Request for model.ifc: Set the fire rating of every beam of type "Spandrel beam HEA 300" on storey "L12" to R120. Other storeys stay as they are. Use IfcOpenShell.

First a look at what the model holds.

```python
import ifcopenshell
import ifcopenshell.util.element

model = ifcopenshell.open("model.ifc")
print(model.schema)
storey = next(s for s in model.by_type("IfcBuildingStorey") if s.Name == "L12")
beams = [e for e in ifcopenshell.util.element.get_decomposition(storey) if e.is_a("IfcBeam")]
seen = {}
for e in beams:
    element_type = ifcopenshell.util.element.get_type(e)
    key = (element_type.Name if element_type != e and element_type else None, ifcopenshell.util.element.get_pset(e, "Pset_BeamCommon", "FireRating"))
    seen[key] = seen.get(key, 0) + 1
for (name, value), count in sorted(seen.items(), key=str):
    print(count, "x", name, "|", value)
```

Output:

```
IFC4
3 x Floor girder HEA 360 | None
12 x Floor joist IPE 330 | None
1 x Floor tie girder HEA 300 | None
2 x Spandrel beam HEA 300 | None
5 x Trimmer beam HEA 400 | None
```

```python
import ifcopenshell
import ifcopenshell.api.pset
import ifcopenshell.util.element

model = ifcopenshell.open("model.ifc")

storey = next(s for s in model.by_type("IfcBuildingStorey") if s.Name == "L12")
beams = [e for e in ifcopenshell.util.element.get_decomposition(storey) if e.is_a("IfcBeam")]

count = 0
for e in beams:
    element_type = ifcopenshell.util.element.get_type(e)
    if element_type in (None, e) or element_type.Name != "Spandrel beam HEA 300":
        continue
    # add_pset returns the element's existing set when there is one.
    pset = ifcopenshell.api.pset.add_pset(model, product=e, name="Pset_BeamCommon")
    ifcopenshell.api.pset.edit_pset(model, pset=pset, properties={"FireRating": "R120"})
    count += 1

print(count, "beams updated")

model.write("model_v2.ifc")
```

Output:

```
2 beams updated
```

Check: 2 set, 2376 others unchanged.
